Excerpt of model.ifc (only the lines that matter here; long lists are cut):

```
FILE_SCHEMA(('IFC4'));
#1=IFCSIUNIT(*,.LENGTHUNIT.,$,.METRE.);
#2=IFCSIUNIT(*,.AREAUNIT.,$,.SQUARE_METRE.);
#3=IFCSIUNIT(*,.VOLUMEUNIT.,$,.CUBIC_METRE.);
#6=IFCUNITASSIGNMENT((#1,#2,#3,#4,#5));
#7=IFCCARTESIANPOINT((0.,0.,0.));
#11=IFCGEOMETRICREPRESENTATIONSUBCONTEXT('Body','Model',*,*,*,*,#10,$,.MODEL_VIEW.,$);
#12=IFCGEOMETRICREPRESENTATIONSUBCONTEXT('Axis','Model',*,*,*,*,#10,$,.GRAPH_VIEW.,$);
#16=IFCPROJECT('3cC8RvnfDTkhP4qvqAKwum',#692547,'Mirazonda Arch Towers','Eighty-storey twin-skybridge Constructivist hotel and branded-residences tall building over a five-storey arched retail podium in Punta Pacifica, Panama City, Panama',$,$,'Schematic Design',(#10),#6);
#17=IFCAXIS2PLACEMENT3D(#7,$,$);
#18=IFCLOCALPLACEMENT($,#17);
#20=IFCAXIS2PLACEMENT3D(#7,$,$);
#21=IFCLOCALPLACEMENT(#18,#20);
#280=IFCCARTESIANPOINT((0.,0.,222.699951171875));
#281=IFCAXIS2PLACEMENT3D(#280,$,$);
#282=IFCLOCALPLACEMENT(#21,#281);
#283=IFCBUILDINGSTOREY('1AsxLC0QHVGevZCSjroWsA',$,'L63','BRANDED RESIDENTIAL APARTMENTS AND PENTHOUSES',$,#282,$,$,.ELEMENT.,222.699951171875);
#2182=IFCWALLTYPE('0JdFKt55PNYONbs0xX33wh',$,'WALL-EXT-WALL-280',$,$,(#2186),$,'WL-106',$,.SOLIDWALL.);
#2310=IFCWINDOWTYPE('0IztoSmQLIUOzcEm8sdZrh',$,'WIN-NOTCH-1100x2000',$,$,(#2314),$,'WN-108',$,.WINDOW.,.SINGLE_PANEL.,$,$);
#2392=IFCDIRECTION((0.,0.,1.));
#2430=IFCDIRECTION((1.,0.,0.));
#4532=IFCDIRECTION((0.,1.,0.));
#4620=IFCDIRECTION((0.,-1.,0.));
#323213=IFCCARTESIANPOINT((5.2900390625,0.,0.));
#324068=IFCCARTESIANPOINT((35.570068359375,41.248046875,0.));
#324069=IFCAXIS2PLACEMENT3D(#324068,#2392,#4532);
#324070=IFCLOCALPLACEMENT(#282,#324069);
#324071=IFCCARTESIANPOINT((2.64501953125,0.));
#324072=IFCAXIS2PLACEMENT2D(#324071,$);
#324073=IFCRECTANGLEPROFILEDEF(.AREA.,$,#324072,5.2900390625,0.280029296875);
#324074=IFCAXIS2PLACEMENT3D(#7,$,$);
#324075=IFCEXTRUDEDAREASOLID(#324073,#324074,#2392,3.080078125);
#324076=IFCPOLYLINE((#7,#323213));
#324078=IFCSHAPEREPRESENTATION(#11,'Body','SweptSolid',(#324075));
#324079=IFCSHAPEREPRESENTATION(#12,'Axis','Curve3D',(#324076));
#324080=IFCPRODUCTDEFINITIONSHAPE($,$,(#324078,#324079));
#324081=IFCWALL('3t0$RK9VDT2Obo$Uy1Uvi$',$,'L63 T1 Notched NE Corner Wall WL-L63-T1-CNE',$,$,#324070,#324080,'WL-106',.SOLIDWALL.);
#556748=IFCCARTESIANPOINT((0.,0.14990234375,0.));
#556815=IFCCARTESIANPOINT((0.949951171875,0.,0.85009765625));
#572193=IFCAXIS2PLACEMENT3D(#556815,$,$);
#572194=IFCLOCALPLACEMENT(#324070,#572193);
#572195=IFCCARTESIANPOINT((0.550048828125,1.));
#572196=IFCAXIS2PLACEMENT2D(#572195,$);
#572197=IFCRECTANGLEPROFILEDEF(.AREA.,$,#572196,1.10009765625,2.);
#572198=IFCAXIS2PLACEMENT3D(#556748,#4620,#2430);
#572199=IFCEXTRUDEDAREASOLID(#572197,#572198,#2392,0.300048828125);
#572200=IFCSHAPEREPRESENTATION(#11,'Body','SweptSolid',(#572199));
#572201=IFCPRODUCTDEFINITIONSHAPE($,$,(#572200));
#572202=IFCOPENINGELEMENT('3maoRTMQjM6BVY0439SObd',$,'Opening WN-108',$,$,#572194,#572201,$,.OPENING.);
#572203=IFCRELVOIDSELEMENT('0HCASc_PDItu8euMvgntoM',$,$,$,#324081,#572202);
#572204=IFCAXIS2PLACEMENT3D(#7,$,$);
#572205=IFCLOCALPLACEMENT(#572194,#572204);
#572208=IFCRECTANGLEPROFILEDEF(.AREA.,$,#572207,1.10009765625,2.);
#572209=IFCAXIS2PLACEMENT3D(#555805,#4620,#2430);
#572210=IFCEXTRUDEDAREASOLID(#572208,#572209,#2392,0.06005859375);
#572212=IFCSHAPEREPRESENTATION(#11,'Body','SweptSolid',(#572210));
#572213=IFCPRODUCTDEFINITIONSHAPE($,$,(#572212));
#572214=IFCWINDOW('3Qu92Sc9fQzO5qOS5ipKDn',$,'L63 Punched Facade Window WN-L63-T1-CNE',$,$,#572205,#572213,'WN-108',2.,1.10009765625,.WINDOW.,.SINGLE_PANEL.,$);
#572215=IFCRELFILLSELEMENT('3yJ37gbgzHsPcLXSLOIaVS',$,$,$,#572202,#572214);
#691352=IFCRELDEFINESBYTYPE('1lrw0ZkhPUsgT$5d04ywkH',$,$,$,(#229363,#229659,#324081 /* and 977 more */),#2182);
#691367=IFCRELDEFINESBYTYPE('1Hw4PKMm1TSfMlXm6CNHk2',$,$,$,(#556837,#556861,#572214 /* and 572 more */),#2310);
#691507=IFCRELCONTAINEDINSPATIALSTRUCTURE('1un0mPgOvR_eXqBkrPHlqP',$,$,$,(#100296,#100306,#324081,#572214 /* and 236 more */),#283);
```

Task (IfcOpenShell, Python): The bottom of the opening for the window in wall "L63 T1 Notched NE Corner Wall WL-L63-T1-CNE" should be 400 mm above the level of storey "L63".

```python
import numpy as np
import ifcopenshell
import ifcopenshell.api.geometry
import ifcopenshell.geom
import ifcopenshell.util.element
import ifcopenshell.util.placement
import ifcopenshell.util.shape
import ifcopenshell.util.unit

model = ifcopenshell.open("model.ifc")
unit_scale = ifcopenshell.util.unit.calculate_unit_scale(model)

window = model.by_guid("3Qu92Sc9fQzO5qOS5ipKDn")
opening = window.FillsVoids[0].RelatingOpeningElement
storey = ifcopenshell.util.element.get_container(window, ifc_class="IfcBuildingStorey")
level = ifcopenshell.util.placement.get_local_placement(storey.ObjectPlacement)[2, 3]

# The opening's origin need not be at the sill, so measure its lowest point.
shape = ifcopenshell.geom.create_shape(ifcopenshell.geom.settings(), opening)
bottom = ifcopenshell.util.shape.get_shape_bottom_elevation(shape, shape.geometry) / unit_scale
dz = level + 0.4 - bottom

shift = np.array([0.0, 0.0, dz])
# The window is placed relative to its opening, so it follows when the opening moves.
matrix = ifcopenshell.util.placement.get_local_placement(opening.ObjectPlacement)
matrix[:3, 3] += shift
ifcopenshell.api.geometry.edit_object_placement(
    model, product=opening, matrix=matrix, is_si=False, should_transform_children=True
)

print(f"moved by {dz * unit_scale:+.3f} m")

model.write("model_edited.ifc")
```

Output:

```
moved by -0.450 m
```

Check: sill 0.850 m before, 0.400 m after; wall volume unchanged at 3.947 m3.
